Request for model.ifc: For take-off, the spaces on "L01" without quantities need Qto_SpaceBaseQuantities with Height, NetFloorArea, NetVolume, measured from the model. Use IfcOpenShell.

First a look at what the model holds.

```python
import ifcopenshell
import ifcopenshell.util.element
import ifcopenshell.util.unit

model = ifcopenshell.open("model.ifc")
print(model.schema)
for unit_type in ("LENGTHUNIT", "AREAUNIT", "VOLUMEUNIT"):
    print(unit_type, ifcopenshell.util.unit.calculate_unit_scale(model, unit_type))
storey = next(s for s in model.by_type("IfcBuildingStorey") if s.Name == "L01")
spaces = [e for e in ifcopenshell.util.element.get_decomposition(storey) if e.is_a("IfcSpace")]
for e in sorted(spaces, key=lambda e: e.id()):
    print(e.id(), e.is_a(), e.Name, list(ifcopenshell.util.element.get_psets(e, qtos_only=True)), sep=" | ")
```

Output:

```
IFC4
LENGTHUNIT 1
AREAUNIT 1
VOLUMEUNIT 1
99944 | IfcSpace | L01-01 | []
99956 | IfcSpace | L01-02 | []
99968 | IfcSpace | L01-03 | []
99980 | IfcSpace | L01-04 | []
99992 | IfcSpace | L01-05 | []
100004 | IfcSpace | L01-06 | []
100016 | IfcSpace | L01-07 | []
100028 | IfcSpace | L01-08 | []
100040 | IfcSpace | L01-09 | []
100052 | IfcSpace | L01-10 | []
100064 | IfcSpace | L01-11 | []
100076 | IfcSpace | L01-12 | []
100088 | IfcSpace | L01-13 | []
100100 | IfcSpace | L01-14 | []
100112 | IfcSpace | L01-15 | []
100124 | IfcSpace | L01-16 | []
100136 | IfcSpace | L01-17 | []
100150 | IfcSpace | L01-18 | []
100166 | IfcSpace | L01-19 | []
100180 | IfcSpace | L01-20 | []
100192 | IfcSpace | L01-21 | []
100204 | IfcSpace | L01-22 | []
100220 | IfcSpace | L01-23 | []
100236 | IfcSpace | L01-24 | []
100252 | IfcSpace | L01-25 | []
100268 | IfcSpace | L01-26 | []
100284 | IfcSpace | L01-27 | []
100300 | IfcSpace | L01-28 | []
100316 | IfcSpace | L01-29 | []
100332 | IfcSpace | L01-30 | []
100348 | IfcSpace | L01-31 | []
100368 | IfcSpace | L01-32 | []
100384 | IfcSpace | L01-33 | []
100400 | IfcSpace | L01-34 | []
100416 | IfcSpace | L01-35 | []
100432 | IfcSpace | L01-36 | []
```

```python
import ifcopenshell
import ifcopenshell.api.pset
import ifcopenshell.geom
import ifcopenshell.util.element
import ifcopenshell.util.shape
import ifcopenshell.util.unit

model = ifcopenshell.open("model.ifc")
unit_scale = ifcopenshell.util.unit.calculate_unit_scale(model)
area_scale = ifcopenshell.util.unit.calculate_unit_scale(model, "AREAUNIT")
volume_scale = ifcopenshell.util.unit.calculate_unit_scale(model, "VOLUMEUNIT")
settings = ifcopenshell.geom.settings()

storey = next(s for s in model.by_type("IfcBuildingStorey") if s.Name == "L01")
spaces = [e for e in ifcopenshell.util.element.get_decomposition(storey) if e.is_a("IfcSpace")]

for e in sorted(spaces, key=lambda e: e.id()):
    if ifcopenshell.util.element.get_psets(e, qtos_only=True, should_inherit=False):
        continue
    # Geometry comes back in metres, in the element's own axes.
    shape = ifcopenshell.geom.create_shape(settings, e)
    values = {
        "Height": ifcopenshell.util.shape.get_z(shape.geometry) / unit_scale,
        "NetFloorArea": ifcopenshell.util.shape.get_footprint_area(shape.geometry) / area_scale,
        "NetVolume": ifcopenshell.util.shape.get_volume(shape.geometry) / volume_scale,
    }
    qto = ifcopenshell.api.pset.add_qto(model, product=e, name="Qto_SpaceBaseQuantities")
    ifcopenshell.api.pset.edit_qto(model, qto=qto, properties=values)
    print(e.id(), {k: round(v, 3) for k, v in values.items()})

model.write("model_edited.ifc")
```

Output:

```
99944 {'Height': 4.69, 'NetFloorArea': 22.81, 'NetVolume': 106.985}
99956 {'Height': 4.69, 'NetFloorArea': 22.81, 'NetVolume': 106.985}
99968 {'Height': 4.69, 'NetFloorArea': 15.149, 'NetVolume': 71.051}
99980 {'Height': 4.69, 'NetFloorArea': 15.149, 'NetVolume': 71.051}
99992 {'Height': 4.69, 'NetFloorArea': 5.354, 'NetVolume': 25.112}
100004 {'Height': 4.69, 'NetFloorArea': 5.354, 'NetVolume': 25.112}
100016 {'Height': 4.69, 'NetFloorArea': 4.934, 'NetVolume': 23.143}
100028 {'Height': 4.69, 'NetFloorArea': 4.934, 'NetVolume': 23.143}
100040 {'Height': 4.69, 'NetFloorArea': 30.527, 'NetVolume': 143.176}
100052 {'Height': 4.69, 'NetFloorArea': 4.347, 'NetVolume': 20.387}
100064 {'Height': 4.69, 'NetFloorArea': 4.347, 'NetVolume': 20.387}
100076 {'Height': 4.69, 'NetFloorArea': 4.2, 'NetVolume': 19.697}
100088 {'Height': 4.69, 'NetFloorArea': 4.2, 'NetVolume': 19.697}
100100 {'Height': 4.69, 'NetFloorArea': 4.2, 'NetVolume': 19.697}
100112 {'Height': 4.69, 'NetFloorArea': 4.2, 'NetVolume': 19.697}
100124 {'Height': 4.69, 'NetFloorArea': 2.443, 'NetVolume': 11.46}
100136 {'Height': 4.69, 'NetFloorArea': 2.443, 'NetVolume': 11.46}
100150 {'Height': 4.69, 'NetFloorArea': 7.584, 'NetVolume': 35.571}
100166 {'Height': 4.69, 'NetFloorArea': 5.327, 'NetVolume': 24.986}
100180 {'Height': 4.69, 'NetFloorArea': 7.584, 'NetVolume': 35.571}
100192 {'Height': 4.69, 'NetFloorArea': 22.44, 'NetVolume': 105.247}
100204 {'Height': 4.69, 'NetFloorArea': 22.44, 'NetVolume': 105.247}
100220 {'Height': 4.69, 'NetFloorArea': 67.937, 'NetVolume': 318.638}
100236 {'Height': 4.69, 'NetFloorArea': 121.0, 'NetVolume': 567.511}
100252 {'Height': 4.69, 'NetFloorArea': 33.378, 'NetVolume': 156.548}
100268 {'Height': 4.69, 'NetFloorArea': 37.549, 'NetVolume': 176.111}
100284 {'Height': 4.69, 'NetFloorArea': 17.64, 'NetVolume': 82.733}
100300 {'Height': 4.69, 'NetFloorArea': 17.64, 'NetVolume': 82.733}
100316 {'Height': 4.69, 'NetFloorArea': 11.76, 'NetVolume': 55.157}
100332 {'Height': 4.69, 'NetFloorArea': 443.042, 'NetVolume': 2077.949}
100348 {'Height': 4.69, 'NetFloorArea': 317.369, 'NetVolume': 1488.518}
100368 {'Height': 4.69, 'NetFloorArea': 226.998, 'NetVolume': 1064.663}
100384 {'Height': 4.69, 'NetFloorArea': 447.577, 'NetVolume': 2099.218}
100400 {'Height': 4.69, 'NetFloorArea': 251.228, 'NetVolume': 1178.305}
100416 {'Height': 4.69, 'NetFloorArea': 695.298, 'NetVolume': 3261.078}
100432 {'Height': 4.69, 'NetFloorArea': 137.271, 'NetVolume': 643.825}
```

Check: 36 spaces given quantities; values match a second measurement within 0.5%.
